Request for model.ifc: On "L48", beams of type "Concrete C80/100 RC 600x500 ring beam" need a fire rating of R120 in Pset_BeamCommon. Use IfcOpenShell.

First a look at what the model holds.

```python
import ifcopenshell
import ifcopenshell.util.element

model = ifcopenshell.open("model.ifc")
print(model.schema)
storey = next(s for s in model.by_type("IfcBuildingStorey") if s.Name == "L48")
beams = [e for e in ifcopenshell.util.element.get_decomposition(storey) if e.is_a("IfcBeam")]
seen = {}
for e in beams:
    element_type = ifcopenshell.util.element.get_type(e)
    key = (element_type.Name if element_type != e and element_type else None, ifcopenshell.util.element.get_pset(e, "Pset_BeamCommon", "FireRating"))
    seen[key] = seen.get(key, 0) + 1
for (name, value), count in sorted(seen.items(), key=str):
    print(count, "x", name, "|", value)
```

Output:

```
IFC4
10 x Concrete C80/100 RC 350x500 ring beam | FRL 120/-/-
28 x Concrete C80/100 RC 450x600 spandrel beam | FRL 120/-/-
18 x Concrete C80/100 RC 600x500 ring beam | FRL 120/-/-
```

```python
import ifcopenshell
import ifcopenshell.api.pset
import ifcopenshell.util.element

model = ifcopenshell.open("model.ifc")

storey = next(s for s in model.by_type("IfcBuildingStorey") if s.Name == "L48")
beams = [e for e in ifcopenshell.util.element.get_decomposition(storey) if e.is_a("IfcBeam")]

count = 0
for e in beams:
    element_type = ifcopenshell.util.element.get_type(e)
    if element_type in (None, e) or element_type.Name != "Concrete C80/100 RC 600x500 ring beam":
        continue
    found = ifcopenshell.util.element.get_pset(e, "Pset_BeamCommon", should_inherit=False)
    if found:
        pset = model.by_id(found["id"])
        if len(ifcopenshell.util.element.get_elements_by_pset(pset)) > 1:
            pset = ifcopenshell.api.pset.unshare_pset(model, products=[e], pset=pset)[0]
    else:
        pset = ifcopenshell.api.pset.add_pset(model, product=e, name="Pset_BeamCommon")
    ifcopenshell.api.pset.edit_pset(model, pset=pset, properties={"FireRating": "R120"})
    count += 1

print(count, "beams updated")

model.write("model_v2.ifc")
```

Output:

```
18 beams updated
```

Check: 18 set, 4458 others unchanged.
